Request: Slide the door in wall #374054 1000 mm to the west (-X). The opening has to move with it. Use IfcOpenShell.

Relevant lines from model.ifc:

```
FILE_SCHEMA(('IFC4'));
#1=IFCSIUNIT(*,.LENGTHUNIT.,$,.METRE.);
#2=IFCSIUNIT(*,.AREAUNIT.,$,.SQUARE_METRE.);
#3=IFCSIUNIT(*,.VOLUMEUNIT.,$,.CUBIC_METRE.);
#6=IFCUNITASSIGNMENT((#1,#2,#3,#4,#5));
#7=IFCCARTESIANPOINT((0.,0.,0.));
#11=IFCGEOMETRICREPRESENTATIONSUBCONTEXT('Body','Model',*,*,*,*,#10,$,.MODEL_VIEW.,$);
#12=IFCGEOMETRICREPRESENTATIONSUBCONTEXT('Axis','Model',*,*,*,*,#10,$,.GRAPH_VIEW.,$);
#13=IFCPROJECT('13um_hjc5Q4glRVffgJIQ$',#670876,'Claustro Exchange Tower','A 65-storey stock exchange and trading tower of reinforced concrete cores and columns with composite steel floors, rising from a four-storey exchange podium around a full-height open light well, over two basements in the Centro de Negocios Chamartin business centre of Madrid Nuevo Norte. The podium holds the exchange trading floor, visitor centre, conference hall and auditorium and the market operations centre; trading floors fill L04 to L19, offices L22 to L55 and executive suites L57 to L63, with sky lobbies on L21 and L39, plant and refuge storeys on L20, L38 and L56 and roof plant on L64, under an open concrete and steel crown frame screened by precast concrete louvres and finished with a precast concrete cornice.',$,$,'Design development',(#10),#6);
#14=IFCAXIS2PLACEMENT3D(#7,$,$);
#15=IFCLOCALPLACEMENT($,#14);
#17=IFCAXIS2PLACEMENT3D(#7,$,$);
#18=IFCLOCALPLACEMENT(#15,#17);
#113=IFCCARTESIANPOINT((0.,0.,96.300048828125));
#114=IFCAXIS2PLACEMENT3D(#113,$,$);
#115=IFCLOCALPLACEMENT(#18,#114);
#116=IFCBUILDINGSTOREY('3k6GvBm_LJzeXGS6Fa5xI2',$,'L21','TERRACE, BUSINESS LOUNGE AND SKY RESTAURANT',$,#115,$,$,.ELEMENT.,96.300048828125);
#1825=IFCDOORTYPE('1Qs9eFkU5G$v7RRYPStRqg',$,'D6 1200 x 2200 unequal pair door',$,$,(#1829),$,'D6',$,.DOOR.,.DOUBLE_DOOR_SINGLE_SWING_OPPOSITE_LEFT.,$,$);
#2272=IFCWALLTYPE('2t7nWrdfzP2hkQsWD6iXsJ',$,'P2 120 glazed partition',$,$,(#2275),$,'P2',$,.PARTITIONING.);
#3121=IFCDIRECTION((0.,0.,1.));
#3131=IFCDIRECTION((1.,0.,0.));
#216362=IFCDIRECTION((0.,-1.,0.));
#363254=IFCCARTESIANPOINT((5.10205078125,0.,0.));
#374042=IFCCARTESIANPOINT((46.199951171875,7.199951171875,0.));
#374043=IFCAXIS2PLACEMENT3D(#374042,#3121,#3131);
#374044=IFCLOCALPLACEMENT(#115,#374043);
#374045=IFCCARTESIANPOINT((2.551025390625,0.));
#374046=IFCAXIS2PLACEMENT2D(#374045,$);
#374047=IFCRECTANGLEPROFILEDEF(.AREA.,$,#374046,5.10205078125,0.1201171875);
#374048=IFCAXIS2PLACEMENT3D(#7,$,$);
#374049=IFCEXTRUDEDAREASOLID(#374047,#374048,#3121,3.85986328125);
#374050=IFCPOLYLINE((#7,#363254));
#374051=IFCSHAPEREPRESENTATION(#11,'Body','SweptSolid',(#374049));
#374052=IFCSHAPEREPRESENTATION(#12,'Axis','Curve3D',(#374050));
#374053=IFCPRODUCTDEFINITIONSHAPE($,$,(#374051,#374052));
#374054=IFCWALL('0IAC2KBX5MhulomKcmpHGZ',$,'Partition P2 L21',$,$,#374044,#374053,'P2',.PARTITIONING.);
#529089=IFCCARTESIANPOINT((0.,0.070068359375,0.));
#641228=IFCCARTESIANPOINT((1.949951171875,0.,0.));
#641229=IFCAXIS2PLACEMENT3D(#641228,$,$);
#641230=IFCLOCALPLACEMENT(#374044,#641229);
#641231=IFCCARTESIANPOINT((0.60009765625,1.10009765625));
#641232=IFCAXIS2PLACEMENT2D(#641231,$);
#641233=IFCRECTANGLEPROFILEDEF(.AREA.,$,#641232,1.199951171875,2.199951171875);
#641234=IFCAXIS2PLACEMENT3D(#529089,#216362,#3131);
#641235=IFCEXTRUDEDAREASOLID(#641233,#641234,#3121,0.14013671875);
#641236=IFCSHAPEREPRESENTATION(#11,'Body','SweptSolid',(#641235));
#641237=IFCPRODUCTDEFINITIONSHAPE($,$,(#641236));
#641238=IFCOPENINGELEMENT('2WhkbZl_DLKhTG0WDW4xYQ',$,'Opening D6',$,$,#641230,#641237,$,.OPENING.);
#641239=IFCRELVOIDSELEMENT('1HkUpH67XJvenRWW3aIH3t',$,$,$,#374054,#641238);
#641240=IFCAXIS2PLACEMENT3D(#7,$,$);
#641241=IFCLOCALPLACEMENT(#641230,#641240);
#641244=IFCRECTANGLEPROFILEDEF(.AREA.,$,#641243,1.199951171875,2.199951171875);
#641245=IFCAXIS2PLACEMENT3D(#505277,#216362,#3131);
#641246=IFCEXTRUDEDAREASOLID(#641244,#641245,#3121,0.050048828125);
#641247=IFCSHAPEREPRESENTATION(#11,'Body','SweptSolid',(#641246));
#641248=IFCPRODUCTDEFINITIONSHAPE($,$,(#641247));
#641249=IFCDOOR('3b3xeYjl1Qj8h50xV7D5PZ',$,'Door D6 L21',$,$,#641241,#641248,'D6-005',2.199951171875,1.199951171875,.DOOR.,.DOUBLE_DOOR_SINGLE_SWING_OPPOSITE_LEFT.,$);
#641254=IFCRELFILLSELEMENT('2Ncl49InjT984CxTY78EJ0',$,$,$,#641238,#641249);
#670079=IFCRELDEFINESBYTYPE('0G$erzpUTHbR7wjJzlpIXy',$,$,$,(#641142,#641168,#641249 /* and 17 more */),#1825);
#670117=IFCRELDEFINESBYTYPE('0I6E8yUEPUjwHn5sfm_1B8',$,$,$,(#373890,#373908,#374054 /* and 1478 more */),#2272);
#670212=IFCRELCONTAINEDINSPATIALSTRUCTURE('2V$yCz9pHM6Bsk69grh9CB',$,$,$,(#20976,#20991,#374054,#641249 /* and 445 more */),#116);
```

```python
import ifcopenshell
import ifcopenshell.api.geometry
import ifcopenshell.util.placement
import ifcopenshell.util.unit

model = ifcopenshell.open("model.ifc")
unit_scale = ifcopenshell.util.unit.calculate_unit_scale(model)

door = model.by_id(641249)
opening = door.FillsVoids[0].RelatingOpeningElement
wall = opening.VoidsElements[0].RelatingBuildingElement

wall_matrix = ifcopenshell.util.placement.get_local_placement(wall.ObjectPlacement)
shift = wall_matrix[:3, 0] * -1 / unit_scale
before = ifcopenshell.util.placement.get_local_placement(door.ObjectPlacement)[:3, 3].copy()

# The door is placed relative to its opening, so it follows when the opening moves.
matrix = ifcopenshell.util.placement.get_local_placement(opening.ObjectPlacement)
matrix[:3, 3] += shift
ifcopenshell.api.geometry.edit_object_placement(
    model, product=opening, matrix=matrix, is_si=False, should_transform_children=True
)

after = ifcopenshell.util.placement.get_local_placement(door.ObjectPlacement)[:3, 3]
print("door moved by", (after - before).round(3) + 0.0)

model.write("model_rev.ifc")
```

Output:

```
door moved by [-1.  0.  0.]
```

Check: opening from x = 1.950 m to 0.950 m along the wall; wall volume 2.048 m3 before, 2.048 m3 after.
